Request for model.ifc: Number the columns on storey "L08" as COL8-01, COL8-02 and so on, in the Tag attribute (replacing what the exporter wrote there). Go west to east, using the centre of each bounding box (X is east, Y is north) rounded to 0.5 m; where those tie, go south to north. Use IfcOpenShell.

First a look at what the model holds.

```python
import ifcopenshell
import ifcopenshell.util.element
import ifcopenshell.util.placement

model = ifcopenshell.open("model.ifc")
print(model.schema)
storey = next(s for s in model.by_type("IfcBuildingStorey") if s.Name == "L08")
columns = [e for e in ifcopenshell.util.element.get_decomposition(storey) if e.is_a("IfcColumn")]
for e in sorted(columns, key=lambda e: e.id()):
    origin = ifcopenshell.util.placement.get_local_placement(e.ObjectPlacement)[:3, 3]
    print(e.id(), e.Tag, e.Name, origin.round(2) + 0.0, sep=" | ")
```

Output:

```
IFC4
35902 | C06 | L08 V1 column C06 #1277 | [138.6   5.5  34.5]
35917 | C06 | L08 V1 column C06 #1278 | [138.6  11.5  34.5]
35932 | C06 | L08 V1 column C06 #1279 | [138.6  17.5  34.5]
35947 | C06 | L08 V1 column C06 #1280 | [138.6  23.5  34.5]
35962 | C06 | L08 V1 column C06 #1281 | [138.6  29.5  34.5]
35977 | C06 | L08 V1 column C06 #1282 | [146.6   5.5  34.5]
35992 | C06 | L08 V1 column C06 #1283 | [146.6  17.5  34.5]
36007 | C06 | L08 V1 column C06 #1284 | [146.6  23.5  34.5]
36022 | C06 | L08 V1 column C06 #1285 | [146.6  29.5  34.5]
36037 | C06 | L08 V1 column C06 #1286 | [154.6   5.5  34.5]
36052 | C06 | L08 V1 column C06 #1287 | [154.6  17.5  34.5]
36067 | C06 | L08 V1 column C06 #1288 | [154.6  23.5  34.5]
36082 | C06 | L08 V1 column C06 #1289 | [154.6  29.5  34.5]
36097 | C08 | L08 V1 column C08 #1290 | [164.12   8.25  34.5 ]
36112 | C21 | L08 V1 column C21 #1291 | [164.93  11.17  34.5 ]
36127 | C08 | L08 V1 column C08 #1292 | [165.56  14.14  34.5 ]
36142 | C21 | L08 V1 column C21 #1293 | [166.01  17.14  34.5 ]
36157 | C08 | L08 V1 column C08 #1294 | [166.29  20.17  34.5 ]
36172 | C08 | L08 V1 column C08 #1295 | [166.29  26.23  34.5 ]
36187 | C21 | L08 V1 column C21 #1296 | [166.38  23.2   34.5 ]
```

```python
import ifcopenshell
import ifcopenshell.geom
import ifcopenshell.util.element
import ifcopenshell.util.shape

model = ifcopenshell.open("model.ifc")
settings = ifcopenshell.geom.settings()
settings.set("use-world-coords", True)


def centre(element):
    shape = ifcopenshell.geom.create_shape(settings, element)
    return ifcopenshell.util.shape.get_bbox_centroid(shape.geometry)


storey = next(s for s in model.by_type("IfcBuildingStorey") if s.Name == "L08")
columns = [e for e in ifcopenshell.util.element.get_decomposition(storey) if e.is_a("IfcColumn")]

# Insertion points can sit at a corner or the storey origin, so sort by the geometry (in metres).
centres = {e: centre(e) for e in columns}
columns.sort(key=lambda e: (round(centres[e][0] / 0.5), centres[e][1]))

for i, e in enumerate(columns, start=1):
    number = f"COL8-{i:02d}"
    e.Tag = number
    print(e.id(), number)

model.write("model-out.ifc")
```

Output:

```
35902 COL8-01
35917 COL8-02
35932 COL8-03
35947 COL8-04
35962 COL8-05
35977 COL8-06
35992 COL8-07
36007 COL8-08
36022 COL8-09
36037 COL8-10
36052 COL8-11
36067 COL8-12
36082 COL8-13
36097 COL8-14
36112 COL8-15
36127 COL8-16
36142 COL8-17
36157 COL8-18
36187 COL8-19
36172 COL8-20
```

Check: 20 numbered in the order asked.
